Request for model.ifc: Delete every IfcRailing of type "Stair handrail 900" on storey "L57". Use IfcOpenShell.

First a look at what the model holds.

```python
import ifcopenshell
import ifcopenshell.util.element

model = ifcopenshell.open("model.ifc")
print(model.schema)
storey = next(s for s in model.by_type("IfcBuildingStorey") if s.Name == "L57")
railings = [e for e in ifcopenshell.util.element.get_decomposition(storey) if e.is_a("IfcRailing")]
seen = {}
for e in railings:
    element_type = ifcopenshell.util.element.get_type(e)
    name = element_type.Name if element_type not in (None, e) else None
    seen[name] = seen.get(name, 0) + 1
for name, count in sorted(seen.items(), key=str):
    print(count, "x", name)
```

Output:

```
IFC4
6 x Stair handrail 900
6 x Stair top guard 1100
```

```python
import ifcopenshell
import ifcopenshell.api.root
import ifcopenshell.util.element

model = ifcopenshell.open("model.ifc")

storey = next(s for s in model.by_type("IfcBuildingStorey") if s.Name == "L57")
railings = [e for e in ifcopenshell.util.element.get_decomposition(storey) if e.is_a("IfcRailing")]
targets = [e for e in railings if (t := ifcopenshell.util.element.get_type(e)) not in (None, e) and t.Name == "Stair handrail 900"]

for e in targets:
    ifcopenshell.api.root.remove_product(model, product=e)
print(len(targets), "removed")

model.write("model_updated.ifc")
```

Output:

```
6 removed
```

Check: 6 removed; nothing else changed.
